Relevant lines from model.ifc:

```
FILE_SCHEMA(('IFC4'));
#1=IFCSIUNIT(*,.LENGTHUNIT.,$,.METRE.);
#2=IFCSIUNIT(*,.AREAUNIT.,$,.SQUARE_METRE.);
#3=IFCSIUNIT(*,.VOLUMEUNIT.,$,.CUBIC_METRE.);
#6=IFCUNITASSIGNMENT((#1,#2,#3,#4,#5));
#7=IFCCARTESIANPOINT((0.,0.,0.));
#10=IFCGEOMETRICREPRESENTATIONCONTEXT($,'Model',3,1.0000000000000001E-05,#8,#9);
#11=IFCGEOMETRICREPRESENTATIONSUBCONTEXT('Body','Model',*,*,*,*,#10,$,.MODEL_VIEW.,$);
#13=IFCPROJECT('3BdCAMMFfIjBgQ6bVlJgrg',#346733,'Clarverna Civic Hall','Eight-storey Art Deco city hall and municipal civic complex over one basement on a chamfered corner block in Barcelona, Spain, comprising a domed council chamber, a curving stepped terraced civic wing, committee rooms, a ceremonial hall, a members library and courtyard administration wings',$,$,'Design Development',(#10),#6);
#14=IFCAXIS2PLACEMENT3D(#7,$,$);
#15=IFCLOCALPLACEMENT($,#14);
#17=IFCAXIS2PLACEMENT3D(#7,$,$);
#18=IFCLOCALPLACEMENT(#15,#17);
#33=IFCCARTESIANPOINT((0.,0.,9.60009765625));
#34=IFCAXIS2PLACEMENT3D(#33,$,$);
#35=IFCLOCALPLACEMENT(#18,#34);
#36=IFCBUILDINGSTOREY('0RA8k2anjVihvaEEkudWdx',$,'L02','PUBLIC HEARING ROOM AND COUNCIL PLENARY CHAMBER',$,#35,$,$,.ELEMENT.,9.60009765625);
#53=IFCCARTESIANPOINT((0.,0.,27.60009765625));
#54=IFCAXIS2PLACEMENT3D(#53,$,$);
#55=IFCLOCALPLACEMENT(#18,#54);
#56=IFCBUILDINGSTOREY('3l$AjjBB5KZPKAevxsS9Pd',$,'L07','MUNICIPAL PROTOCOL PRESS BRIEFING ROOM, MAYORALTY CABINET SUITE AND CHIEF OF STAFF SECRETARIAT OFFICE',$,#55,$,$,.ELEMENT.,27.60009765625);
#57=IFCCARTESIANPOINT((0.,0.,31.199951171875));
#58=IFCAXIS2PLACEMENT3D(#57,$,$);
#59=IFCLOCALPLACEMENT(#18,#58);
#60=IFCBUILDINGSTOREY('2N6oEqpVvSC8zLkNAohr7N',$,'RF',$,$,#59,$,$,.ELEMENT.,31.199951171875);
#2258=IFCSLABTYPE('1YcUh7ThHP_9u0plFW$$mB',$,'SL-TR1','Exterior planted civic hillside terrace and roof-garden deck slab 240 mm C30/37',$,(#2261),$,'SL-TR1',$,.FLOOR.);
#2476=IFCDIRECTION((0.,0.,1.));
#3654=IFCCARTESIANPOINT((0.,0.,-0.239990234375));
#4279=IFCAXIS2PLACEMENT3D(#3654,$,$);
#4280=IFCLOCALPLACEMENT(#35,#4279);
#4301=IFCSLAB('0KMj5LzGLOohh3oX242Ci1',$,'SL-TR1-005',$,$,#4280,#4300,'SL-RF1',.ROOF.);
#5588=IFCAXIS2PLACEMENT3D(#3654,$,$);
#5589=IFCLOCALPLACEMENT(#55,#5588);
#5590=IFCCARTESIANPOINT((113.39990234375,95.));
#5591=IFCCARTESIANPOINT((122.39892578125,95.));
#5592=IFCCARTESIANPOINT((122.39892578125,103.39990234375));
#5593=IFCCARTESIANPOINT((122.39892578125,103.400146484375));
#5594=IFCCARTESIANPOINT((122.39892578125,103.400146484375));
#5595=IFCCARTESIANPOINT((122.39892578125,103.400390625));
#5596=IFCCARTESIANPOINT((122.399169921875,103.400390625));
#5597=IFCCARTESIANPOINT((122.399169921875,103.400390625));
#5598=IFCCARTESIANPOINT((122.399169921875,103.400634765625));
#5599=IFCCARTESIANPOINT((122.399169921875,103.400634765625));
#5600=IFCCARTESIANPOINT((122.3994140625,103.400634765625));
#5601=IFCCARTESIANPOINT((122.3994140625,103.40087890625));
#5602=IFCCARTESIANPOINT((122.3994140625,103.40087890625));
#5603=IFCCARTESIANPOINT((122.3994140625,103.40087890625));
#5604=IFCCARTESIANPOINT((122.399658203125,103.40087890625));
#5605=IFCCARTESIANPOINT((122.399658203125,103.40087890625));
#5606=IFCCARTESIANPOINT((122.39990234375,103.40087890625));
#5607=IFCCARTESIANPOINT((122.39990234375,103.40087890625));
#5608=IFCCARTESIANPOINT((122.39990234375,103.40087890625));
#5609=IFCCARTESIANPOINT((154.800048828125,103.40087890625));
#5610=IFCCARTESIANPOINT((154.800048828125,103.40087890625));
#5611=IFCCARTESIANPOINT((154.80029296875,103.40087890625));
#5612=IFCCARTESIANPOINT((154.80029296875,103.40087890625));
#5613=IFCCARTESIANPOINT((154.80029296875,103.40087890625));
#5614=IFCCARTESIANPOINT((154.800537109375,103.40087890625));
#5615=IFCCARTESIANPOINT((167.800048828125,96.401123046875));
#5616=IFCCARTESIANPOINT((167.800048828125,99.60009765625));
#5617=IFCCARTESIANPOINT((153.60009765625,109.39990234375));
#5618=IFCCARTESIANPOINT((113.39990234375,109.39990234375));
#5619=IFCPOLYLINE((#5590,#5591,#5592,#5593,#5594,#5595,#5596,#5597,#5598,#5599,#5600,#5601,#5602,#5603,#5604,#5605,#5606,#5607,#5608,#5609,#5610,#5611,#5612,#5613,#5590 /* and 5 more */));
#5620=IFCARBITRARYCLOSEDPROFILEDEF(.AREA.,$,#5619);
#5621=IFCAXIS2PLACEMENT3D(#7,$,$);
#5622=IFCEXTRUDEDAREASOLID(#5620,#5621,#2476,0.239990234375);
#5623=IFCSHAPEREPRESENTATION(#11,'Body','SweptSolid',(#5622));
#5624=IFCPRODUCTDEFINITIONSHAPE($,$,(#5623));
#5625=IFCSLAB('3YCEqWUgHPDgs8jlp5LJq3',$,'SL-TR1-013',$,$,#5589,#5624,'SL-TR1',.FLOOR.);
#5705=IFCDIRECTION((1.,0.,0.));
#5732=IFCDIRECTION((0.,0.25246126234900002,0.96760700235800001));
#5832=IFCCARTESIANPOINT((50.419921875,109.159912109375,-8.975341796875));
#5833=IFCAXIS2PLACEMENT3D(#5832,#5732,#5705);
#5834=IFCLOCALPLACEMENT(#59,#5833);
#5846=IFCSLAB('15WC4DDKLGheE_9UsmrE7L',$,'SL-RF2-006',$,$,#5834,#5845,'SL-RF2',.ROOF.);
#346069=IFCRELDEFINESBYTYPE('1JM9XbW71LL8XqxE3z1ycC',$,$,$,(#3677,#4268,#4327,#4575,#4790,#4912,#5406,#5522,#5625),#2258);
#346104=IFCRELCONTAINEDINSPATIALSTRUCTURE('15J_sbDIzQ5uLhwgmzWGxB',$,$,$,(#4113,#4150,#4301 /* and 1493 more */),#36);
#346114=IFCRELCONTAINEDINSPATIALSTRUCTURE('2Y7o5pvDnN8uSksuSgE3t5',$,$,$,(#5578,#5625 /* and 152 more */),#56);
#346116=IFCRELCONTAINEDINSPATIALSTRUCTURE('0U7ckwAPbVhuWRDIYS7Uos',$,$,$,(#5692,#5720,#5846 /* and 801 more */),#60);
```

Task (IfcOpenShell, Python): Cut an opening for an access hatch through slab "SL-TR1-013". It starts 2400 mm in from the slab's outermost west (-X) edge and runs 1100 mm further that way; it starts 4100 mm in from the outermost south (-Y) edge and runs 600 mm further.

```python
import numpy as np
import ifcopenshell
import ifcopenshell.api.feature
import ifcopenshell.api.geometry
import ifcopenshell.api.root
import ifcopenshell.geom
import ifcopenshell.util.placement
import ifcopenshell.util.representation
import ifcopenshell.util.shape
import ifcopenshell.util.unit

model = ifcopenshell.open("model.ifc")
unit_scale = ifcopenshell.util.unit.calculate_unit_scale(model)
settings = ifcopenshell.geom.settings()


def volume(element):
    """Net volume in cubic metres, openings subtracted."""
    shape = ifcopenshell.geom.create_shape(settings, element)
    return ifcopenshell.util.shape.get_volume(shape.geometry)


slab = model.by_id(5625)
before = volume(slab)

# Extent in the slab's own axes, in metres. The edges named are its -X and -Y sides.
slab_shape = ifcopenshell.geom.create_shape(settings, slab)
vertices = ifcopenshell.util.shape.get_vertices(slab_shape.geometry)
x_min, y_min, bottom = vertices.min(axis=0)
top = vertices[:, 2].max()

opening = ifcopenshell.api.root.create_entity(model, ifc_class="IfcOpeningElement", name="Access hatch opening", predefined_type="OPENING")
context = ifcopenshell.util.representation.get_context(model, "Model", "Body", "MODEL_VIEW")
width, depth = 1.1, 0.6
outline = [(0.0, 0.0), (width, 0.0), (width, depth), (0.0, depth), (0.0, 0.0)]
# Overshoot both faces by 50 mm so the cut is clean.
shape = ifcopenshell.api.geometry.add_slab_representation(
    model, context=context, depth=top - bottom + 0.1, polyline=outline
)
ifcopenshell.api.geometry.assign_representation(model, product=opening, representation=shape)

matrix = ifcopenshell.util.placement.get_local_placement(slab.ObjectPlacement)
matrix[:, 3] = matrix @ np.append(np.array([x_min + 2.4, y_min + 4.1, bottom - 0.05]) / unit_scale, 1.0)
ifcopenshell.api.geometry.edit_object_placement(model, product=opening, matrix=matrix, is_si=False)
ifcopenshell.api.feature.add_feature(model, feature=opening, element=slab)

after = volume(slab)

print(f"slab volume {before:.3f} -> {after:.3f} m3")

model.write("model_updated.ifc")
```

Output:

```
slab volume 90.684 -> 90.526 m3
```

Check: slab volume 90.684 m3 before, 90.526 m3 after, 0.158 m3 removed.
